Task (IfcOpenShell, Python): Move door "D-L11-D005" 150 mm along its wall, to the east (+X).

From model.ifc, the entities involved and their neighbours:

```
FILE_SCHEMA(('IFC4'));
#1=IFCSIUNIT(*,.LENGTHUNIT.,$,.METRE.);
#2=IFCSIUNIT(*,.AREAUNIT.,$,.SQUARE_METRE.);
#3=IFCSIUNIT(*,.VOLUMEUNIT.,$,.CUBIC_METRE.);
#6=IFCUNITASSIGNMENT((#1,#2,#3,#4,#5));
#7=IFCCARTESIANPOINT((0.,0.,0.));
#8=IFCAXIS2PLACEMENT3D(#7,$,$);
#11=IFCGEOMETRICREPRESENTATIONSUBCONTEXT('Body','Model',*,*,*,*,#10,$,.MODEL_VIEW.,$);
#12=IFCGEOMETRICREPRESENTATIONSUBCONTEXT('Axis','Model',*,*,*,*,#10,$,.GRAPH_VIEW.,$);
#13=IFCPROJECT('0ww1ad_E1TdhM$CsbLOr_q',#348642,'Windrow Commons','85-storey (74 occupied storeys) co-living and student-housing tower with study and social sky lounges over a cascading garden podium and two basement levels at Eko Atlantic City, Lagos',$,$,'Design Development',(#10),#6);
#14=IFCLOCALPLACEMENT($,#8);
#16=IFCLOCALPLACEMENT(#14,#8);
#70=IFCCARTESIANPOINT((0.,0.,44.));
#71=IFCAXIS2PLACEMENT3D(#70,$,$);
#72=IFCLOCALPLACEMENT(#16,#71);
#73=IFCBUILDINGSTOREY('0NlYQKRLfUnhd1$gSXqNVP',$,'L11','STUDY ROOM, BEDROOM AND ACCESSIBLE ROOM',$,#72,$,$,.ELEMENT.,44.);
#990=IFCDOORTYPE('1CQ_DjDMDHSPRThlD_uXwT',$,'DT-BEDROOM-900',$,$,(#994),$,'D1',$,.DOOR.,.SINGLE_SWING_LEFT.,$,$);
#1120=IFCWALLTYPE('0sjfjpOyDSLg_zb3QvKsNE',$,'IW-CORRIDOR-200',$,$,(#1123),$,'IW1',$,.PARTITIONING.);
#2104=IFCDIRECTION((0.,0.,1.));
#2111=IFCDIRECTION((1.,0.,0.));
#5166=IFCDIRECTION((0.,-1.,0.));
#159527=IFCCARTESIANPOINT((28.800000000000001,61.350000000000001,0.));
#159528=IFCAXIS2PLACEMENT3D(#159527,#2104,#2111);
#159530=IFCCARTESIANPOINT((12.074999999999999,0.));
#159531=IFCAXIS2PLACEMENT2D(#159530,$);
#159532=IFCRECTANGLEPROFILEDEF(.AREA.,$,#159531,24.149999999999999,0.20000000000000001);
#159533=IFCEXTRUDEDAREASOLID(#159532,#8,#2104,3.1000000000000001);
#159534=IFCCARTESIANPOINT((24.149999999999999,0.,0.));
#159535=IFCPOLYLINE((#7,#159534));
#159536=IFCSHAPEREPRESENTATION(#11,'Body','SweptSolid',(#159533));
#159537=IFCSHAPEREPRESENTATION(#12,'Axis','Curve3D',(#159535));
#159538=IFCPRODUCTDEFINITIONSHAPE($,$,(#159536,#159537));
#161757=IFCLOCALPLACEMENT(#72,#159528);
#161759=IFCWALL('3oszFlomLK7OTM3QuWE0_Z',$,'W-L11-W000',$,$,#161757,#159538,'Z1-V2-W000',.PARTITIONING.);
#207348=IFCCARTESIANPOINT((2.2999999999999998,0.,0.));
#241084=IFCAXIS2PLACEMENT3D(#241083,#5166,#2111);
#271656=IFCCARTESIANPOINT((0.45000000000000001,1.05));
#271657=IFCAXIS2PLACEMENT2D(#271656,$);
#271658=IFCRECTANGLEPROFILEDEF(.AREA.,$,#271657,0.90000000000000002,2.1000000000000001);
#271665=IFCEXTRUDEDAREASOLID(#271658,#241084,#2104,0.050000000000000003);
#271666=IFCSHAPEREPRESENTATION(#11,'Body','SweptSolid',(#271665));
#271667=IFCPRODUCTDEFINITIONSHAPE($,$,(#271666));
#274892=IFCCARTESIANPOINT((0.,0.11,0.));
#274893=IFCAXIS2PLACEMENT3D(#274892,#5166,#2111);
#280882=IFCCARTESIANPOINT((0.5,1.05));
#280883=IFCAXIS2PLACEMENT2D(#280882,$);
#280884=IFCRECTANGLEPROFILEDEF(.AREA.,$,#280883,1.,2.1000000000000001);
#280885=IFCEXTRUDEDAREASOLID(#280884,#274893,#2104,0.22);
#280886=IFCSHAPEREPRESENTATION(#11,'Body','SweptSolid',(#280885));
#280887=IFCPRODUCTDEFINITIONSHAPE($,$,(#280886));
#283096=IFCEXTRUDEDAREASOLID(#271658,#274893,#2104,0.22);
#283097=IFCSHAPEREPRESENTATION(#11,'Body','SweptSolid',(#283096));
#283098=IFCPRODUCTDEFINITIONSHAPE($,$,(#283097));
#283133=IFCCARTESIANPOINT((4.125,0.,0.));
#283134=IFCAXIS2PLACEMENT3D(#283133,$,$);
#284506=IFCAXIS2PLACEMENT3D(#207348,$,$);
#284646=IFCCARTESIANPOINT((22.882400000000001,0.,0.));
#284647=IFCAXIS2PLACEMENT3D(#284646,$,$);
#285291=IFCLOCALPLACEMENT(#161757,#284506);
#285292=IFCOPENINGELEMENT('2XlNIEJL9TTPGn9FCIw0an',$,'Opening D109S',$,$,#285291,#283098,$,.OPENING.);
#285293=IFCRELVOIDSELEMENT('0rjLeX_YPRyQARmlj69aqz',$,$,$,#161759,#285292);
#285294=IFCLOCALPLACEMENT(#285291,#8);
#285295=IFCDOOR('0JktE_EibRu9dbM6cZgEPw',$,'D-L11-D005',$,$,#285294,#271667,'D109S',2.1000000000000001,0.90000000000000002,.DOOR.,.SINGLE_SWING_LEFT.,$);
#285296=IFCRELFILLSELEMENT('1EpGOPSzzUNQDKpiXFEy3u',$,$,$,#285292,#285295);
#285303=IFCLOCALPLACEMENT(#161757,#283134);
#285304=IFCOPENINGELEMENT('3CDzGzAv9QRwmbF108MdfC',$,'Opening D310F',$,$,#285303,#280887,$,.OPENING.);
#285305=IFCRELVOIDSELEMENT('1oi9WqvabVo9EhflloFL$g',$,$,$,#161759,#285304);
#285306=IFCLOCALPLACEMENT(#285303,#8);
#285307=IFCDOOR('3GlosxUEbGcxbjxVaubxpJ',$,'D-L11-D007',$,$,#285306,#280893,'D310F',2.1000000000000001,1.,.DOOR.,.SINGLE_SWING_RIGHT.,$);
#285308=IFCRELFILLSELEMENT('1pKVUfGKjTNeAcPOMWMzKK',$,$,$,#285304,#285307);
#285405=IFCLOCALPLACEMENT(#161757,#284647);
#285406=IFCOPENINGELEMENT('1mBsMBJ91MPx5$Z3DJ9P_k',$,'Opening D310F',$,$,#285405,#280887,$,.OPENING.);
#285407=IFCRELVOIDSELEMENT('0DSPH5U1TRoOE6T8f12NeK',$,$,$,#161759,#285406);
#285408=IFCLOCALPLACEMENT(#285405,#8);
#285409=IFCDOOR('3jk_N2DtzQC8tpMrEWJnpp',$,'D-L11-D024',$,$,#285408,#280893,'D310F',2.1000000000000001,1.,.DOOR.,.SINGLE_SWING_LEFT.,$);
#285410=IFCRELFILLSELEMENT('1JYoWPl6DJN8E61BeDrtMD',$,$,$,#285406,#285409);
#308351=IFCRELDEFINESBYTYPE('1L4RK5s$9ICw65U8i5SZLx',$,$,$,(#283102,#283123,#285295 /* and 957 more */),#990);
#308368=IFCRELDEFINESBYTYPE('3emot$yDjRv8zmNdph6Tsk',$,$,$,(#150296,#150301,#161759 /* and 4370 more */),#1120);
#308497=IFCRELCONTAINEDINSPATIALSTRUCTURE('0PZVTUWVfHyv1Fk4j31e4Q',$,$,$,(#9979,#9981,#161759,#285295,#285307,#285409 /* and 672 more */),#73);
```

```python
import ifcopenshell
import ifcopenshell.api.geometry
import ifcopenshell.util.placement

model = ifcopenshell.open("model.ifc")

door = model.by_id(285295)
opening = door.FillsVoids[0].RelatingOpeningElement
wall = opening.VoidsElements[0].RelatingBuildingElement

wall_matrix = ifcopenshell.util.placement.get_local_placement(wall.ObjectPlacement)
shift = wall_matrix[:3, 0] * 0.15
before = ifcopenshell.util.placement.get_local_placement(door.ObjectPlacement)[:3, 3].copy()

# The door is placed relative to its opening, so it follows when the opening moves.
matrix = ifcopenshell.util.placement.get_local_placement(opening.ObjectPlacement)
matrix[:3, 3] += shift
ifcopenshell.api.geometry.edit_object_placement(
    model, product=opening, matrix=matrix, is_si=False, should_transform_children=True
)

after = ifcopenshell.util.placement.get_local_placement(door.ObjectPlacement)[:3, 3]
print("door moved by", (after - before).round(3) + 0.0)

model.write("model_edited.ifc")
```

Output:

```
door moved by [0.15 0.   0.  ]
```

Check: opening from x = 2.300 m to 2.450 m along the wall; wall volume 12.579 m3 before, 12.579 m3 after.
